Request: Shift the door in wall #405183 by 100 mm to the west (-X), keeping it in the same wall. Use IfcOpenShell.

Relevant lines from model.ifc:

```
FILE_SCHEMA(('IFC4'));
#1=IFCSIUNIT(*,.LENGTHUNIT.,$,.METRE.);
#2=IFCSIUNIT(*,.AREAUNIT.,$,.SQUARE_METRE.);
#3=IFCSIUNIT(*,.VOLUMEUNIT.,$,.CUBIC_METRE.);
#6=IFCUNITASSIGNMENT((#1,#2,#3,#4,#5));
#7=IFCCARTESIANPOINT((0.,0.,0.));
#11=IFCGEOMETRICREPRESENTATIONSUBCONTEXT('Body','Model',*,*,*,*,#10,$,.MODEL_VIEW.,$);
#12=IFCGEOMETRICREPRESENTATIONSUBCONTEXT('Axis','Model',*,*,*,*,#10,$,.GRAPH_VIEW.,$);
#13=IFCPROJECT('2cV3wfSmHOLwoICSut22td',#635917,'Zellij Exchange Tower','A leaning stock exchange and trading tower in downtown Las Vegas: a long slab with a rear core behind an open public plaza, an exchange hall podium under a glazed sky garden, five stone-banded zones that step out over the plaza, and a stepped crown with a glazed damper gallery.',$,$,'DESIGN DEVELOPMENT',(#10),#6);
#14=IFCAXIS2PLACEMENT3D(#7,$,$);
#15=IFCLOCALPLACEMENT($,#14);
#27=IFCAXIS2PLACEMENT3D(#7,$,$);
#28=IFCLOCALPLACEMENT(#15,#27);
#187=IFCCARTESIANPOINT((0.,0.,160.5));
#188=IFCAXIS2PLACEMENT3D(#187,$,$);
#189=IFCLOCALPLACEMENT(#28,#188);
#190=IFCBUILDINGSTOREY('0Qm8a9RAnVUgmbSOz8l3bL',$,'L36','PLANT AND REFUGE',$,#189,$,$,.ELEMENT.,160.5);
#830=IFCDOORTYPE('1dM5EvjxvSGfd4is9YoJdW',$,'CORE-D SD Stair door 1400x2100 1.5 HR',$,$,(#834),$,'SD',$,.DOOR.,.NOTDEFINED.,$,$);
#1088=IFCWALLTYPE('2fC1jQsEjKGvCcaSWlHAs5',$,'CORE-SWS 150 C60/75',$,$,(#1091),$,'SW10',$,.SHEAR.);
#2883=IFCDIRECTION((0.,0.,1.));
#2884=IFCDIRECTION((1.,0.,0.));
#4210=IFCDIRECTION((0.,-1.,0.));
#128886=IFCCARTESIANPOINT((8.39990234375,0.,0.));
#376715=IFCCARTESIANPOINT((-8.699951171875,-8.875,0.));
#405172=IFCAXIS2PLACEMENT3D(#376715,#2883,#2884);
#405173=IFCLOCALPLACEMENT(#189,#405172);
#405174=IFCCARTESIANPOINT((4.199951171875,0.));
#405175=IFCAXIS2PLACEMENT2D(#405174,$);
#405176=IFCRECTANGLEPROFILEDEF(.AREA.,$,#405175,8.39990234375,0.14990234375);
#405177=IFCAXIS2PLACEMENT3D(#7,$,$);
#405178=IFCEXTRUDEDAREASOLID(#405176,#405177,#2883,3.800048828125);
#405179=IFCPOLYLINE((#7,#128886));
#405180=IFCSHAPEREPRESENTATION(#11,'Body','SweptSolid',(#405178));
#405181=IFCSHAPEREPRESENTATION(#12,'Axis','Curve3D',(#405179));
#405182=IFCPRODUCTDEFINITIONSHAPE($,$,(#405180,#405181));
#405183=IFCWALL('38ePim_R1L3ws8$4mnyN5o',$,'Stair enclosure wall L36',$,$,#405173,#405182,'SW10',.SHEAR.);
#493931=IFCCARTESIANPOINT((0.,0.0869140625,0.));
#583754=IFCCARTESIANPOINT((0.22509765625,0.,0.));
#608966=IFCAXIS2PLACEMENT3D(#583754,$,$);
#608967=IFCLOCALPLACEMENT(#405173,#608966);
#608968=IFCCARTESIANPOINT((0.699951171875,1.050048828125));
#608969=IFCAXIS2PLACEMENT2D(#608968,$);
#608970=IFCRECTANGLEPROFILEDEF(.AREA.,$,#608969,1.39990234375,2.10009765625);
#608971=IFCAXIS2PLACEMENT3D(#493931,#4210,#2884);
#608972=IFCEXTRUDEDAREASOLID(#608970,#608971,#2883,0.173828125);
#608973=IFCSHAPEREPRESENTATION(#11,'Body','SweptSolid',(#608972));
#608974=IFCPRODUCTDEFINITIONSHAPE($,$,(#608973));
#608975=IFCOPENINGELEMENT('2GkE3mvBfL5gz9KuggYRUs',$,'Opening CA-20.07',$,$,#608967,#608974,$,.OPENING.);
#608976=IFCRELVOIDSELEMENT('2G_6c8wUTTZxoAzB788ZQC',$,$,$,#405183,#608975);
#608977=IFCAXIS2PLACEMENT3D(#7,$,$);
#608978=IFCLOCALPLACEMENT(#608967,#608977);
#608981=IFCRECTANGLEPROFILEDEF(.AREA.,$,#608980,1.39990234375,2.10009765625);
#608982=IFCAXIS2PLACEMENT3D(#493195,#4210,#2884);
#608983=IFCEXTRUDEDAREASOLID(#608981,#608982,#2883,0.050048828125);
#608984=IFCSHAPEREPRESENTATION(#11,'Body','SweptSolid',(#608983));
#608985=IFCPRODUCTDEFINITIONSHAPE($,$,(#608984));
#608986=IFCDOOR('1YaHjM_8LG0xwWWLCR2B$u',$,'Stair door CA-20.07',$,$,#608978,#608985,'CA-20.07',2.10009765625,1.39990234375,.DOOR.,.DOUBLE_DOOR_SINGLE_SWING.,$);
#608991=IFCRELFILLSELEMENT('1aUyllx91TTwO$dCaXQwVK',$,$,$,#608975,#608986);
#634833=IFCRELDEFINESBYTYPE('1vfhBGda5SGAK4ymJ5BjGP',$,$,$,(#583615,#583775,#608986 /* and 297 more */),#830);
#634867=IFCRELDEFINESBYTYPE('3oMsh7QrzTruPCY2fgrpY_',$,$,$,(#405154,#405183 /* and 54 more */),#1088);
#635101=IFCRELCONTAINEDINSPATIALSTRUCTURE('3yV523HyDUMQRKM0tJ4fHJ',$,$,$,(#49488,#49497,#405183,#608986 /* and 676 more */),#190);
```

```python
import ifcopenshell
import ifcopenshell.api.geometry
import ifcopenshell.util.placement

model = ifcopenshell.open("model.ifc")

door = model.by_guid("1YaHjM_8LG0xwWWLCR2B$u")
opening = door.FillsVoids[0].RelatingOpeningElement
wall = opening.VoidsElements[0].RelatingBuildingElement

wall_matrix = ifcopenshell.util.placement.get_local_placement(wall.ObjectPlacement)
shift = wall_matrix[:3, 0] * -0.1
before = ifcopenshell.util.placement.get_local_placement(door.ObjectPlacement)[:3, 3].copy()

# The door is placed relative to its opening, so it follows when the opening moves.
matrix = ifcopenshell.util.placement.get_local_placement(opening.ObjectPlacement)
matrix[:3, 3] += shift
ifcopenshell.api.geometry.edit_object_placement(
    model, product=opening, matrix=matrix, is_si=False, should_transform_children=True
)

after = ifcopenshell.util.placement.get_local_placement(door.ObjectPlacement)[:3, 3]
print("door moved by", (after - before).round(3) + 0.0)

model.write("model_edited.ifc")
```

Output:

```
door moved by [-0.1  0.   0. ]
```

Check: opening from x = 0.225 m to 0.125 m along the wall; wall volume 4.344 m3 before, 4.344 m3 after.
